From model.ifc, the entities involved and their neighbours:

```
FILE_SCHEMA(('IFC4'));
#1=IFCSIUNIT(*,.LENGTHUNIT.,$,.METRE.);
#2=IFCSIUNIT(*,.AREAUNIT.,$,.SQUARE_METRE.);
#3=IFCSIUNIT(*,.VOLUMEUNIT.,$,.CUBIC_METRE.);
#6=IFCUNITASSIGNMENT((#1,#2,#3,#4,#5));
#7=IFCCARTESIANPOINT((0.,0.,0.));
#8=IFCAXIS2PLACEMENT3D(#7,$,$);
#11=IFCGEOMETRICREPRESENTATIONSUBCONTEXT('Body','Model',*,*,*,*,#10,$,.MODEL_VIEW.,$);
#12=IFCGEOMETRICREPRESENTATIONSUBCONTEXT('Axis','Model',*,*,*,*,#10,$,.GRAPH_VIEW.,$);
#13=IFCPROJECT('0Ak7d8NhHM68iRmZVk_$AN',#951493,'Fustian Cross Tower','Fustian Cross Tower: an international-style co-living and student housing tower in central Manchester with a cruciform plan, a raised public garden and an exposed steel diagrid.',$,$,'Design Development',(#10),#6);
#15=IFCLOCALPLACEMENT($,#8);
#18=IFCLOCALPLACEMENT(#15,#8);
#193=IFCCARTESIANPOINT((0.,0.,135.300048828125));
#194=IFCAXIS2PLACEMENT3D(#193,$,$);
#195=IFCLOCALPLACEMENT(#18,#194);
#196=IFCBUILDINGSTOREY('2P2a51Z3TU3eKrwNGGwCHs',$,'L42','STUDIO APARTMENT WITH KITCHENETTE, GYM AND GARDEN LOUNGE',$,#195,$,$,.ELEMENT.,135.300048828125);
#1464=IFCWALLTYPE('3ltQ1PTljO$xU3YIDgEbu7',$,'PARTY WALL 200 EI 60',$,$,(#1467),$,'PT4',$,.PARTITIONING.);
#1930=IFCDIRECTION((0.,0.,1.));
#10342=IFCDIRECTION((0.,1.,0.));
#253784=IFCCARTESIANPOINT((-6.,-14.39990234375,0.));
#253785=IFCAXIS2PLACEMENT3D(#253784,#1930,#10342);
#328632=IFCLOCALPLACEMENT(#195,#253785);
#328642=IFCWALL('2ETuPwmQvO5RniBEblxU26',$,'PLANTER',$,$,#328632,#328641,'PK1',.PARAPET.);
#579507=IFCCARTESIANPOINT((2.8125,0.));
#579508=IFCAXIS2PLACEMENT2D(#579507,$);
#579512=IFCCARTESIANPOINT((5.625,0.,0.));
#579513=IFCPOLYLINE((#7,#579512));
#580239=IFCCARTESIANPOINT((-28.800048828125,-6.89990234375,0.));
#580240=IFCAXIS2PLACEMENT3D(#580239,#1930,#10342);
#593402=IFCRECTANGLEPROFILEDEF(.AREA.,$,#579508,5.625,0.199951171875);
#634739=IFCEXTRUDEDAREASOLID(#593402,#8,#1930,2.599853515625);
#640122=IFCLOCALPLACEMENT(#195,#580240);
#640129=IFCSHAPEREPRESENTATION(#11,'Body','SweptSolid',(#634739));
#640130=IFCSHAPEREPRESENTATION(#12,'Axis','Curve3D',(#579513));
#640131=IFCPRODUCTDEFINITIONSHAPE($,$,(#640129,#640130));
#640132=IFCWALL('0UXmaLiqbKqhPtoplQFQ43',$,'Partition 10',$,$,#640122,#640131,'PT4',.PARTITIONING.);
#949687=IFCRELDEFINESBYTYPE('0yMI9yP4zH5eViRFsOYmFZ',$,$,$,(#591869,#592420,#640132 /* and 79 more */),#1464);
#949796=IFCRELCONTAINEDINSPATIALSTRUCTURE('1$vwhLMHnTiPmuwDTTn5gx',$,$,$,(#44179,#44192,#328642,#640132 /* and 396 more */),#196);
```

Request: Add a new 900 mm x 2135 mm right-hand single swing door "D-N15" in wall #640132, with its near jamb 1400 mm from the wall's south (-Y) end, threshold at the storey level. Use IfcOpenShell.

```python
import numpy as np
import ifcopenshell
import ifcopenshell.api.feature
import ifcopenshell.api.geometry
import ifcopenshell.api.root
import ifcopenshell.api.spatial
import ifcopenshell.geom
import ifcopenshell.util.element
import ifcopenshell.util.placement
import ifcopenshell.util.representation
import ifcopenshell.util.shape
import ifcopenshell.util.unit

model = ifcopenshell.open("model.ifc")
unit_scale = ifcopenshell.util.unit.calculate_unit_scale(model)
settings = ifcopenshell.geom.settings()


def volume(element):
    """Net volume in cubic metres, openings subtracted."""
    shape = ifcopenshell.geom.create_shape(settings, element)
    return ifcopenshell.util.shape.get_volume(shape.geometry)


wall = model.by_guid("0UXmaLiqbKqhPtoplQFQ43")
storey = ifcopenshell.util.element.get_container(wall, ifc_class="IfcBuildingStorey")
context = ifcopenshell.util.representation.get_context(model, "Model", "Body", "MODEL_VIEW")
before = volume(wall)

width, height, from_end, sill = 0.9, 2.135, 1.4, 0.0  # metres

# The wall runs along its own X axis, and the end named is its -X end.
wall_shape = ifcopenshell.geom.create_shape(settings, wall)
x, y, z = ifcopenshell.util.shape.get_vertices(wall_shape.geometry).T
start = x.min() + from_end
face, thickness = float(y.min()), float(y.max() - y.min())
wall_matrix = ifcopenshell.util.placement.get_local_placement(wall.ObjectPlacement)
level = ifcopenshell.util.placement.get_local_placement(storey.ObjectPlacement)[2, 3]


def in_wall(x, y):
    """Placement at x, y metres in the wall's axes, at sill height."""
    matrix = wall_matrix.copy()
    matrix[:, 3] = wall_matrix @ np.array([x / unit_scale, y / unit_scale, 0.0, 1.0])
    matrix[2, 3] = level + sill / unit_scale
    return matrix


# Opening: a box that overshoots both wall faces by 50 mm.
opening = ifcopenshell.api.root.create_entity(model, ifc_class="IfcOpeningElement", predefined_type="OPENING")
box = ifcopenshell.api.geometry.add_wall_representation(
    model, context=context, length=width, height=height, thickness=thickness + 0.1
)
ifcopenshell.api.geometry.assign_representation(model, product=opening, representation=box)
ifcopenshell.api.geometry.edit_object_placement(model, product=opening, matrix=in_wall(start, face - 0.05), is_si=False)
ifcopenshell.api.feature.add_feature(model, feature=opening, element=wall)

door = ifcopenshell.api.root.create_entity(model, ifc_class="IfcDoor", name="D-N15", predefined_type="DOOR")
door.OverallWidth, door.OverallHeight = width / unit_scale, height / unit_scale
door.OperationType = "SINGLE_SWING_RIGHT"
body = ifcopenshell.api.geometry.add_door_representation(
    model,
    context=context,
    overall_width=door.OverallWidth,
    overall_height=door.OverallHeight,
    operation_type="SINGLE_SWING_RIGHT",
    lining_properties={"LiningDepth": thickness / unit_scale, "ThresholdDepth": thickness / unit_scale},
)
ifcopenshell.api.geometry.assign_representation(model, product=door, representation=body)
ifcopenshell.api.spatial.assign_container(model, products=[door], relating_structure=storey)
ifcopenshell.api.feature.add_filling(model, opening=opening, element=door)

# The lining spans the wall, so the door starts at the wall face.
ifcopenshell.api.geometry.edit_object_placement(model, product=door, matrix=in_wall(start, face), is_si=False)

after = volume(wall)

print(f"wall volume {before:.3f} -> {after:.3f} m3")

model.write("model_updated.ifc")
```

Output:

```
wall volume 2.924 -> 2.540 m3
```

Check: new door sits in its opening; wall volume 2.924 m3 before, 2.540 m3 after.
